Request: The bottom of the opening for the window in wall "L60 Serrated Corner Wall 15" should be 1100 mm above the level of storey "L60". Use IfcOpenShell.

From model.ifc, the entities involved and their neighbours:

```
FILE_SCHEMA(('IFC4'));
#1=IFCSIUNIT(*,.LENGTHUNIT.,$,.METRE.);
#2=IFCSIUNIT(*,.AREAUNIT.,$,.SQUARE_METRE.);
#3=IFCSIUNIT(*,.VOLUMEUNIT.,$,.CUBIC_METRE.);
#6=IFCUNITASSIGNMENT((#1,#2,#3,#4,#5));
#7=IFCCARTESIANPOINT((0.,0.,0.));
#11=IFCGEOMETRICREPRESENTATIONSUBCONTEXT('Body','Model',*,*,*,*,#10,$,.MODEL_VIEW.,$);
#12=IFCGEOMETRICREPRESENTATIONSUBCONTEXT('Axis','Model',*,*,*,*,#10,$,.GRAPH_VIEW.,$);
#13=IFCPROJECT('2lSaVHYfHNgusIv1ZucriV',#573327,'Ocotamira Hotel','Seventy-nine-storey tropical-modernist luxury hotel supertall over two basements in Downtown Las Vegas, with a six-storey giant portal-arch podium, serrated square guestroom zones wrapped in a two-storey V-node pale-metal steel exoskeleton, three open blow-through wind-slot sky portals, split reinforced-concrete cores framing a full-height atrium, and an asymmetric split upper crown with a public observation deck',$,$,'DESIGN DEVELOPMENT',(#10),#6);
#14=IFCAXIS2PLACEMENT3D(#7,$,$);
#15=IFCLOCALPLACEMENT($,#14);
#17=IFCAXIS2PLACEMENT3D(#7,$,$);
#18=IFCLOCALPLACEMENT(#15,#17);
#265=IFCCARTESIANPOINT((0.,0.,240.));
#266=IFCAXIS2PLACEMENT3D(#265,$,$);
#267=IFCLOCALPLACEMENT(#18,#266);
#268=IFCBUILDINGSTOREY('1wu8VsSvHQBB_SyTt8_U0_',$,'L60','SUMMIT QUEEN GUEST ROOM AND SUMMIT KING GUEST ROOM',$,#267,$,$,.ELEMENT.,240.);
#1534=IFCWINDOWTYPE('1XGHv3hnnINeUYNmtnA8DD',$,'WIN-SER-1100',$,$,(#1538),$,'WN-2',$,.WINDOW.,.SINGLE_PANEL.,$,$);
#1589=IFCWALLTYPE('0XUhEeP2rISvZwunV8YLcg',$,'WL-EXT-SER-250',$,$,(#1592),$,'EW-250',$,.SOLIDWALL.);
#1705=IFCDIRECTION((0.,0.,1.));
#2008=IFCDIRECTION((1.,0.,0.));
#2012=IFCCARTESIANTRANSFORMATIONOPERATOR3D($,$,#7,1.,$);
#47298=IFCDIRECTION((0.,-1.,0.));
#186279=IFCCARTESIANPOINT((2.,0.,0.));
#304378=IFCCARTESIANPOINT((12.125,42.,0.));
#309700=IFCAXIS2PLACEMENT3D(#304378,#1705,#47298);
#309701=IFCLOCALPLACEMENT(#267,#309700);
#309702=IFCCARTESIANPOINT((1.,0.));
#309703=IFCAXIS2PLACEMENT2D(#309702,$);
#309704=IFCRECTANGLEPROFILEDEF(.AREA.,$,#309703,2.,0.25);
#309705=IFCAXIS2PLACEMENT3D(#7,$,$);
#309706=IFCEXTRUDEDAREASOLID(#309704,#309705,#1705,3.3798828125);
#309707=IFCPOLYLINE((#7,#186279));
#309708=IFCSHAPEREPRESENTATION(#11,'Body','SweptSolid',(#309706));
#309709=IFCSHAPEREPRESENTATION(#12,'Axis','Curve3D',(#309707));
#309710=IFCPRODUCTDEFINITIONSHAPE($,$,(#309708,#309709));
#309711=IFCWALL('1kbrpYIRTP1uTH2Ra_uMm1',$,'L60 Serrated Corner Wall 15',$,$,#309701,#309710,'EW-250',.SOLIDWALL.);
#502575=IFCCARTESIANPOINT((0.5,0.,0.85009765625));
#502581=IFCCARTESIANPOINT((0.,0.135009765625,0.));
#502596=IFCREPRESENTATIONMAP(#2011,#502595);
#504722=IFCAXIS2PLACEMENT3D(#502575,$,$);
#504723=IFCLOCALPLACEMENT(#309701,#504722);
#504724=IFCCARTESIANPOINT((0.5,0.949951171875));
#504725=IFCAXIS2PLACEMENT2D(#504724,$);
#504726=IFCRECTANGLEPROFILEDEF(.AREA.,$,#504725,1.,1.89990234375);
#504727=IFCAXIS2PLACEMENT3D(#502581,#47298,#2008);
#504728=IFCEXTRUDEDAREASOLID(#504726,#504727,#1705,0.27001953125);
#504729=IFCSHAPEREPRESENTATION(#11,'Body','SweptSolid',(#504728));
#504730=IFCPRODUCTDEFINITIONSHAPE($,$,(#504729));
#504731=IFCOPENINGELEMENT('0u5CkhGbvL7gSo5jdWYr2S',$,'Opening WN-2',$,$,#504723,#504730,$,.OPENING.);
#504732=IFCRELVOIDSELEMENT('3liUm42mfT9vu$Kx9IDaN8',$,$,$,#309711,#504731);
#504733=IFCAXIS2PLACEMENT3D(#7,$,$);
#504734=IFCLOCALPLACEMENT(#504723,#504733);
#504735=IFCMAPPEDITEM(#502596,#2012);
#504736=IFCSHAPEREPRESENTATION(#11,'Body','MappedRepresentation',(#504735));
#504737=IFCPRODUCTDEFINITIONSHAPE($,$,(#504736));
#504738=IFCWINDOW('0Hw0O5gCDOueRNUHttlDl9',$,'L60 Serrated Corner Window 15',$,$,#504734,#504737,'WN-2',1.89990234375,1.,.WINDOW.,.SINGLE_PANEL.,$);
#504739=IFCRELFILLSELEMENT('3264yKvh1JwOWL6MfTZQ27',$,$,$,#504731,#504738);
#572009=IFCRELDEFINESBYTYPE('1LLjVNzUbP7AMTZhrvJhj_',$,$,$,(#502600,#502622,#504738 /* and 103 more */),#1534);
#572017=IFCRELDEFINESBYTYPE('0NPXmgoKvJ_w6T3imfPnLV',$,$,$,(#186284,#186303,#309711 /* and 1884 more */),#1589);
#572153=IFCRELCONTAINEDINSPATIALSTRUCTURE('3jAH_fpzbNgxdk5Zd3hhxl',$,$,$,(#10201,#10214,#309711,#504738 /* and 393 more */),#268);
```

```python
import numpy as np
import ifcopenshell
import ifcopenshell.api.geometry
import ifcopenshell.geom
import ifcopenshell.util.element
import ifcopenshell.util.placement
import ifcopenshell.util.shape
import ifcopenshell.util.unit

model = ifcopenshell.open("model.ifc")
unit_scale = ifcopenshell.util.unit.calculate_unit_scale(model)

window = model.by_guid("0Hw0O5gCDOueRNUHttlDl9")
opening = window.FillsVoids[0].RelatingOpeningElement
storey = ifcopenshell.util.element.get_container(window, ifc_class="IfcBuildingStorey")
level = ifcopenshell.util.placement.get_local_placement(storey.ObjectPlacement)[2, 3]

# The opening's origin need not be at the sill, so measure its lowest point.
shape = ifcopenshell.geom.create_shape(ifcopenshell.geom.settings(), opening)
bottom = ifcopenshell.util.shape.get_shape_bottom_elevation(shape, shape.geometry) / unit_scale
dz = level + 1.1 / unit_scale - bottom

shift = np.array([0.0, 0.0, dz])
# The window is placed relative to its opening, so it follows when the opening moves.
matrix = ifcopenshell.util.placement.get_local_placement(opening.ObjectPlacement)
matrix[:3, 3] += shift
ifcopenshell.api.geometry.edit_object_placement(
    model, product=opening, matrix=matrix, is_si=False, should_transform_children=True
)

print(f"moved by {dz * unit_scale:+.3f} m")

model.write("model_rev.ifc")
```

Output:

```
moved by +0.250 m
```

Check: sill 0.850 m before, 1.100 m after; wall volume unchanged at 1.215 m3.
